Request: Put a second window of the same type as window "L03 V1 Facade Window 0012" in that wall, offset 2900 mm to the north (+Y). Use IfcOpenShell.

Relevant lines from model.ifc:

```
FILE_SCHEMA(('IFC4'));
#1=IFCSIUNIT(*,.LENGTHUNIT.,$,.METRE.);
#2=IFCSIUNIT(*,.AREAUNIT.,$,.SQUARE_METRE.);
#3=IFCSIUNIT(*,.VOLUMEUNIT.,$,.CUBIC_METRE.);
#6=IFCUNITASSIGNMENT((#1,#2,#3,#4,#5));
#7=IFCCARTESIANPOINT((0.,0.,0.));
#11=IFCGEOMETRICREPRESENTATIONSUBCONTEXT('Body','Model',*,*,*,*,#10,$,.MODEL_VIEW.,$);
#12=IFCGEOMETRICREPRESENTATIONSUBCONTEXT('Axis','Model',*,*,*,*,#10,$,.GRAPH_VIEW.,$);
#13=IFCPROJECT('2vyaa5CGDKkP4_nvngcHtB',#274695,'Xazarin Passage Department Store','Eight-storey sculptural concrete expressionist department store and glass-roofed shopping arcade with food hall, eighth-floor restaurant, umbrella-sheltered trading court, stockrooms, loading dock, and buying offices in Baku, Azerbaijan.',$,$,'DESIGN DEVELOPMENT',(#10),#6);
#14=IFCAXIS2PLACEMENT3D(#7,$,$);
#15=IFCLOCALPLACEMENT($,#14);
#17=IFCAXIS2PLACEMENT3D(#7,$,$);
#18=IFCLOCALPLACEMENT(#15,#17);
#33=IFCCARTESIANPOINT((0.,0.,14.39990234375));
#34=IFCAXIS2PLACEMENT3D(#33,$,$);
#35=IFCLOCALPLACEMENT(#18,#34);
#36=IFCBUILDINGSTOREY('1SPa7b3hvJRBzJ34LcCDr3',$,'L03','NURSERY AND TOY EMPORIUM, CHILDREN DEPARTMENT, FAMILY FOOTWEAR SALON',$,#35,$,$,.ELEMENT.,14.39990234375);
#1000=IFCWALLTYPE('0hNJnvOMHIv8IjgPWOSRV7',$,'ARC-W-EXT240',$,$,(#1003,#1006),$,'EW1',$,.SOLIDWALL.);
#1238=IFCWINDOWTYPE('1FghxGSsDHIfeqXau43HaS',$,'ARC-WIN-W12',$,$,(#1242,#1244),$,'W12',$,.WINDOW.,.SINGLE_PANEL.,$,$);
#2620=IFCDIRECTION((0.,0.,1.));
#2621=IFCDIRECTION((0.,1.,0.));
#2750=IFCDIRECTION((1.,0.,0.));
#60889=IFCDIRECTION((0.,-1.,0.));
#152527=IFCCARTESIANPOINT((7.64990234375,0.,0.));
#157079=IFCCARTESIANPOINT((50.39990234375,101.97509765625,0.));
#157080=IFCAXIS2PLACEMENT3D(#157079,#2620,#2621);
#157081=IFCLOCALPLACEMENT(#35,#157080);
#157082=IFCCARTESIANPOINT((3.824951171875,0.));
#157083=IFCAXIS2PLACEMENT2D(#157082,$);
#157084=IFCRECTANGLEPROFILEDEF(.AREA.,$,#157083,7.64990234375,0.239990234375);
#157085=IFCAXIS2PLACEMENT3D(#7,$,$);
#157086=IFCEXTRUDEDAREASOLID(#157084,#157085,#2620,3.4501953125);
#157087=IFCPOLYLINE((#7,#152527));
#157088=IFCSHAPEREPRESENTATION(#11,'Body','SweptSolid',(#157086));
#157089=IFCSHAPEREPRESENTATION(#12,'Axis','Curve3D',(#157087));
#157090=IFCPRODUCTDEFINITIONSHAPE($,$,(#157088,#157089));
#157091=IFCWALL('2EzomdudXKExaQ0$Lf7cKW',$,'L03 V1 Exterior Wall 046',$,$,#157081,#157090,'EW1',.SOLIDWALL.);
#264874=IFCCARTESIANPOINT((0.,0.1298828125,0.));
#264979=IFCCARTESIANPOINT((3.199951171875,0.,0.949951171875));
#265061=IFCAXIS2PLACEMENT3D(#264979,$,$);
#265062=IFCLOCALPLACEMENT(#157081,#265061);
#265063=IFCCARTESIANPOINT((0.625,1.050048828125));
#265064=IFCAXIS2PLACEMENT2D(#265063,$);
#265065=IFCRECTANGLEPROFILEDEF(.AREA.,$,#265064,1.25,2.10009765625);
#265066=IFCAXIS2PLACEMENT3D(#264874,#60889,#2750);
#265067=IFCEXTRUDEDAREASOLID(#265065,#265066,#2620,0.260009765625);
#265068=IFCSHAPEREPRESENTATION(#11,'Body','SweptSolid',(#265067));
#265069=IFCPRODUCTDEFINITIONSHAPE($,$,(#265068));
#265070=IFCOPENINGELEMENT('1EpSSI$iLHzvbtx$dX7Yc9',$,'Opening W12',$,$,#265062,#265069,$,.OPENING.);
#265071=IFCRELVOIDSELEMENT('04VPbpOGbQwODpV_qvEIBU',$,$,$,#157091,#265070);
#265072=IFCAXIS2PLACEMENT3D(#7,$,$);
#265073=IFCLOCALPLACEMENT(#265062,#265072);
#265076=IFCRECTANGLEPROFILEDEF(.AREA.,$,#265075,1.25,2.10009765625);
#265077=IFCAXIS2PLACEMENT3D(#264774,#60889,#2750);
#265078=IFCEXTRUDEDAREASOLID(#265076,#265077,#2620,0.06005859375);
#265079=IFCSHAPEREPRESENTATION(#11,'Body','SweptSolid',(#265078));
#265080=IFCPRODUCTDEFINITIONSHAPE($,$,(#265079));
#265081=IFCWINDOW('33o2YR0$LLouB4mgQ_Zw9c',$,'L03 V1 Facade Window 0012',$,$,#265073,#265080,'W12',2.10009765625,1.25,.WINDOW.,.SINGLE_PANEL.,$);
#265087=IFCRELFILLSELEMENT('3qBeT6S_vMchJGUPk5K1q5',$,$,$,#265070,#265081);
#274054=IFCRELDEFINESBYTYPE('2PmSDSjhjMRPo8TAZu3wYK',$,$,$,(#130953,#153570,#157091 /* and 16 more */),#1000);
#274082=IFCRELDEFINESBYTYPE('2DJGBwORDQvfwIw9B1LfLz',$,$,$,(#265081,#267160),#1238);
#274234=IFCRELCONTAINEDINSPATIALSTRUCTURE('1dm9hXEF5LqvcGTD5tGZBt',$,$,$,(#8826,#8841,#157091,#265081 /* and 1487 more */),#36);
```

```python
import ifcopenshell
import ifcopenshell.api.feature
import ifcopenshell.api.geometry
import ifcopenshell.api.root
import ifcopenshell.geom
import ifcopenshell.util.element
import ifcopenshell.util.placement
import ifcopenshell.util.shape
import ifcopenshell.util.unit

model = ifcopenshell.open("model.ifc")
unit_scale = ifcopenshell.util.unit.calculate_unit_scale(model)
settings = ifcopenshell.geom.settings()


def volume(element):
    """Net volume in cubic metres, openings subtracted."""
    shape = ifcopenshell.geom.create_shape(settings, element)
    return ifcopenshell.util.shape.get_volume(shape.geometry)


window = model.by_guid("33o2YR0$LLouB4mgQ_Zw9c")
opening = window.FillsVoids[0].RelatingOpeningElement
wall = opening.VoidsElements[0].RelatingBuildingElement
before = volume(wall)
shift = ifcopenshell.util.placement.get_local_placement(wall.ObjectPlacement)[:3, 0] * 2.9 / unit_scale

# copy_class copies the void relationship, type, container and properties, but no geometry.
new_opening = ifcopenshell.api.root.copy_class(model, product=opening)
new_opening.Representation = ifcopenshell.util.element.copy_deep(
    model, opening.Representation, exclude=["IfcGeometricRepresentationContext", "IfcRepresentationMap"]
)
new_window = ifcopenshell.api.root.copy_class(model, product=window)
new_window.Representation = ifcopenshell.util.element.copy_deep(
    model, window.Representation, exclude=["IfcGeometricRepresentationContext", "IfcRepresentationMap"]
)
new_window.Tag = None
ifcopenshell.api.feature.add_filling(model, opening=new_opening, element=new_window)

for old, new in ((opening, new_opening), (window, new_window)):
    matrix = ifcopenshell.util.placement.get_local_placement(old.ObjectPlacement)
    matrix[:3, 3] += shift
    ifcopenshell.api.geometry.edit_object_placement(model, product=new, matrix=matrix, is_si=False)

after = volume(wall)

print(f"wall volume {before:.3f} -> {after:.3f} m3")

model.write("model_rev.ifc")
```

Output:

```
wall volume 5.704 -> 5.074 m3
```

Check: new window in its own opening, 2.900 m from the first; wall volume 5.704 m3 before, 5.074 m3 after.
